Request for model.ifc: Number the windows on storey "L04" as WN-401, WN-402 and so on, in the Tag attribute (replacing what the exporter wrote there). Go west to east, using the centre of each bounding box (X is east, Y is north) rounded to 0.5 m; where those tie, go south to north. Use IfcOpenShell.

First a look at what the model holds.

```python
import ifcopenshell
import ifcopenshell.util.element
import ifcopenshell.util.placement

model = ifcopenshell.open("model.ifc")
print(model.schema)
storey = next(s for s in model.by_type("IfcBuildingStorey") if s.Name == "L04")
windows = [e for e in ifcopenshell.util.element.get_decomposition(storey) if e.is_a("IfcWindow")]
for e in sorted(windows, key=lambda e: e.id()):
    origin = ifcopenshell.util.placement.get_local_placement(e.ObjectPlacement)[:3, 3]
    print(e.id(), e.Tag, e.Name, origin.round(2) + 0.0, sep=" | ")
```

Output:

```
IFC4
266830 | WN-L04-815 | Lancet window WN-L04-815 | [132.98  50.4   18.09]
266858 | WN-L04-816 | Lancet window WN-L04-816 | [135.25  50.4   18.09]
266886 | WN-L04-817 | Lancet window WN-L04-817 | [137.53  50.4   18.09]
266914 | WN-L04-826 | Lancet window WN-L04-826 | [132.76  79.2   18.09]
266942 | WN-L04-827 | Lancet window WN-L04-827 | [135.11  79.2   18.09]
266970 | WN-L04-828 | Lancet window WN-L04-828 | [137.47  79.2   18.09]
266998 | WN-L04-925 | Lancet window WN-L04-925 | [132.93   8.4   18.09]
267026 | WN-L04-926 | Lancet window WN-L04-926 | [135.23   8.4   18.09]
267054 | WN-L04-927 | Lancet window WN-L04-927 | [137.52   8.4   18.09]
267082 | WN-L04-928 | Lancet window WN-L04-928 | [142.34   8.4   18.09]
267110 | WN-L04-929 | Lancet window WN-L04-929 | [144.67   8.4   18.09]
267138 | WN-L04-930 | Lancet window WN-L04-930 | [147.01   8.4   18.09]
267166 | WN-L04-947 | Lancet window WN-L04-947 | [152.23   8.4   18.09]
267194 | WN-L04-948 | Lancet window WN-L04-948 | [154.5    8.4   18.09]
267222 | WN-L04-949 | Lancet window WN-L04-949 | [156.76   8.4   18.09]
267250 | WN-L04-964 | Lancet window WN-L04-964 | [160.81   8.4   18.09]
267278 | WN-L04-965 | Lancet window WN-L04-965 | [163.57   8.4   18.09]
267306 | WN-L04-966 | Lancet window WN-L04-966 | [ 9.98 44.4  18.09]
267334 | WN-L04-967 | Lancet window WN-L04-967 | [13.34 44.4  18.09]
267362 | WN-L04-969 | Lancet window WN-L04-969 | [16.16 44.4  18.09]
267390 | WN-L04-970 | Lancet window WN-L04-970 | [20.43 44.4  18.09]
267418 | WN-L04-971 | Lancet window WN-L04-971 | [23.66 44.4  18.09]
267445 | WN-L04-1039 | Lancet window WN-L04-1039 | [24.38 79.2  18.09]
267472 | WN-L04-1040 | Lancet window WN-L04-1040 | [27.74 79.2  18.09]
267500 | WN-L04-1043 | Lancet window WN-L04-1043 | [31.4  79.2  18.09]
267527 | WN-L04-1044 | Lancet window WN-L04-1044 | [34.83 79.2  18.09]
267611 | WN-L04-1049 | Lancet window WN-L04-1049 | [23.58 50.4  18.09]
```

```python
import ifcopenshell
import ifcopenshell.geom
import ifcopenshell.util.element
import ifcopenshell.util.shape

model = ifcopenshell.open("model.ifc")
settings = ifcopenshell.geom.settings()
settings.set("use-world-coords", True)


def centre(element):
    shape = ifcopenshell.geom.create_shape(settings, element)
    return ifcopenshell.util.shape.get_bbox_centroid(shape.geometry)


storey = next(s for s in model.by_type("IfcBuildingStorey") if s.Name == "L04")
windows = [e for e in ifcopenshell.util.element.get_decomposition(storey) if e.is_a("IfcWindow")]

# Insertion points can sit at a corner or the storey origin, so sort by the geometry (in metres).
centres = {e: centre(e) for e in windows}
windows.sort(key=lambda e: (round(centres[e][0] / 0.5), centres[e][1]))

for i, e in enumerate(windows, start=1):
    number = f"WN-4{i:02d}"
    e.Tag = number
    print(e.id(), number)

model.write("model_edited.ifc")
```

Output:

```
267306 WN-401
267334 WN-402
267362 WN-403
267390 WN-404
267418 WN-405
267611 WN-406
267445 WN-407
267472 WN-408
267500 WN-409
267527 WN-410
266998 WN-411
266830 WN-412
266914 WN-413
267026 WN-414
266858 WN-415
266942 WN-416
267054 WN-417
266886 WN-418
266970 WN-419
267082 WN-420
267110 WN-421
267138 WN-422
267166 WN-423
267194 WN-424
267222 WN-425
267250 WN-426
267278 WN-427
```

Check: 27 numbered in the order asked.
